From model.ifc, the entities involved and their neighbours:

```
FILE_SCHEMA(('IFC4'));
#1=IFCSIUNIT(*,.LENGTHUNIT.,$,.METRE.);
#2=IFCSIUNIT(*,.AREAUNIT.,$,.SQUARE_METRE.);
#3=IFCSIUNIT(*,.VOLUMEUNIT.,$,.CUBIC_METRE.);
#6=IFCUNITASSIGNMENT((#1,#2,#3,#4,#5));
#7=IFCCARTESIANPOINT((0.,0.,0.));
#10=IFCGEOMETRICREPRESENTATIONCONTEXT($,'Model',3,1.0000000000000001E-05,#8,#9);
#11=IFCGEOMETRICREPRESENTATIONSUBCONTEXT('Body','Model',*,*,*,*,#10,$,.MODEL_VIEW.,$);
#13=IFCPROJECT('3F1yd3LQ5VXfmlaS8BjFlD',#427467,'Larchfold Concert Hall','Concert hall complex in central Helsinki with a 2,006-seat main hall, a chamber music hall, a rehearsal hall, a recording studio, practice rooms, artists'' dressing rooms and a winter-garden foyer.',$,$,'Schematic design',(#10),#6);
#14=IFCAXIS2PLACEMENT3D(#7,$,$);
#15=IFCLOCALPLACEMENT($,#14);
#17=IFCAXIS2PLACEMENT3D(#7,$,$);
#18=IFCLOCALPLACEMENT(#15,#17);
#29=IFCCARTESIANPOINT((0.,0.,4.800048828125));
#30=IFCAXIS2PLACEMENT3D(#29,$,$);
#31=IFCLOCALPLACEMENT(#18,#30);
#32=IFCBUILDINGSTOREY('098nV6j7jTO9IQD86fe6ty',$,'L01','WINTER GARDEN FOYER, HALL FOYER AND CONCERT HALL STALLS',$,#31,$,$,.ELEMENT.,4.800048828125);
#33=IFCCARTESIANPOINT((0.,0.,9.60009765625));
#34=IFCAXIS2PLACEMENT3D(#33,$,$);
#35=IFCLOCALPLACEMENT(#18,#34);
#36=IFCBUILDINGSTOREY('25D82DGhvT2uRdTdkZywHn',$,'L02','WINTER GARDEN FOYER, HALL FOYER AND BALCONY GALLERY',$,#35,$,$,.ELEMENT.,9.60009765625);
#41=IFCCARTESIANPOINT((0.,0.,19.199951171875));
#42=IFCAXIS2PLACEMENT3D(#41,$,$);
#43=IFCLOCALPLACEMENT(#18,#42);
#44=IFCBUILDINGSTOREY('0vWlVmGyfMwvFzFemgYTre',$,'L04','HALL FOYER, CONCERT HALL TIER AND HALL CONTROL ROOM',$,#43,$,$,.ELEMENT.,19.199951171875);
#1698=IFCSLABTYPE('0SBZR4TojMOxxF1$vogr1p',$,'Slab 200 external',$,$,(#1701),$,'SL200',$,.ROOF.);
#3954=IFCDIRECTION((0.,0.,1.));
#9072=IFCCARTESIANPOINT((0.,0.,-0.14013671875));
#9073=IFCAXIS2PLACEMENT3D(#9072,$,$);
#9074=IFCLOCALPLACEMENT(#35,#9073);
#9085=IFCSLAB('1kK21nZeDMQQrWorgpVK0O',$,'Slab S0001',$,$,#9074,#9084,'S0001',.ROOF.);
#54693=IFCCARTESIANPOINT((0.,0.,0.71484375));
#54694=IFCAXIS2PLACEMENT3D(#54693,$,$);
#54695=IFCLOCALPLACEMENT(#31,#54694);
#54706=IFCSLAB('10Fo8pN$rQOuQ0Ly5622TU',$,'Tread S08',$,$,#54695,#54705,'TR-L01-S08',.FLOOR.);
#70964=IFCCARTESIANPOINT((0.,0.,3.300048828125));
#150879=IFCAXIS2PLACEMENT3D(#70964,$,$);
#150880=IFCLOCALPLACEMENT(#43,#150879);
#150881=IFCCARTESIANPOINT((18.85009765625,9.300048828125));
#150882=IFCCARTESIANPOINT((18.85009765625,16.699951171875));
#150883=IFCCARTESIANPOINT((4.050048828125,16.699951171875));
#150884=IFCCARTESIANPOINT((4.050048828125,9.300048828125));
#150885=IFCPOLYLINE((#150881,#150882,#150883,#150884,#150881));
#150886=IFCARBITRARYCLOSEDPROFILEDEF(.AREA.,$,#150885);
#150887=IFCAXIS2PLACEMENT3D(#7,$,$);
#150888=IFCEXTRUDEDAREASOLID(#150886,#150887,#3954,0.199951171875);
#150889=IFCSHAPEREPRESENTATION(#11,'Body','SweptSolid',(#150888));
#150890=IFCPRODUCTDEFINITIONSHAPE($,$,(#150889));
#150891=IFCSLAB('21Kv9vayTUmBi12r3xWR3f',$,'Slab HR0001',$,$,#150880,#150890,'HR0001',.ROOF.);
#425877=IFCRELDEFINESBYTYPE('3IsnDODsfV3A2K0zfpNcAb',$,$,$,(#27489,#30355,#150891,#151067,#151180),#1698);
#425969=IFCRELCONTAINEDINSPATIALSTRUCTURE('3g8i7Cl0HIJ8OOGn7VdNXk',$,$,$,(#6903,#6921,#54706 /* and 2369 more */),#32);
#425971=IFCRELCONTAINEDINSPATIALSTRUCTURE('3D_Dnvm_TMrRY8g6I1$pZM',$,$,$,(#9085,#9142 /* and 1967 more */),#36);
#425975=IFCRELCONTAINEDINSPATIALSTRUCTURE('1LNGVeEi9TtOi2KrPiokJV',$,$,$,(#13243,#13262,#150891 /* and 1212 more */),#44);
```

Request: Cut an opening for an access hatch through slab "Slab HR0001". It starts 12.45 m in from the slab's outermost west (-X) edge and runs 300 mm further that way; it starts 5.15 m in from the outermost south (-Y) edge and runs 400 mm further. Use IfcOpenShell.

```python
import numpy as np
import ifcopenshell
import ifcopenshell.api.feature
import ifcopenshell.api.geometry
import ifcopenshell.api.root
import ifcopenshell.geom
import ifcopenshell.util.placement
import ifcopenshell.util.representation
import ifcopenshell.util.shape
import ifcopenshell.util.unit

model = ifcopenshell.open("model.ifc")
unit_scale = ifcopenshell.util.unit.calculate_unit_scale(model)
settings = ifcopenshell.geom.settings()


def volume(element):
    """Net volume in cubic metres, openings subtracted."""
    shape = ifcopenshell.geom.create_shape(settings, element)
    return ifcopenshell.util.shape.get_volume(shape.geometry)


slab = model.by_guid("21Kv9vayTUmBi12r3xWR3f")
before = volume(slab)

# Extent in the slab's own axes, in metres. The edges named are its -X and -Y sides.
slab_shape = ifcopenshell.geom.create_shape(settings, slab)
vertices = ifcopenshell.util.shape.get_vertices(slab_shape.geometry)
x_min, y_min, bottom = vertices.min(axis=0)
top = vertices[:, 2].max()

opening = ifcopenshell.api.root.create_entity(model, ifc_class="IfcOpeningElement", name="Access hatch opening", predefined_type="OPENING")
context = ifcopenshell.util.representation.get_context(model, "Model", "Body", "MODEL_VIEW")
width, depth = 0.3, 0.4
outline = [(0.0, 0.0), (width, 0.0), (width, depth), (0.0, depth), (0.0, 0.0)]
# Overshoot both faces by 50 mm so the cut is clean.
shape = ifcopenshell.api.geometry.add_slab_representation(
    model, context=context, depth=top - bottom + 0.1, polyline=outline
)
ifcopenshell.api.geometry.assign_representation(model, product=opening, representation=shape)

matrix = ifcopenshell.util.placement.get_local_placement(slab.ObjectPlacement)
matrix[:, 3] = matrix @ np.append(np.array([x_min + 12.45, y_min + 5.15, bottom - 0.05]) / unit_scale, 1.0)
ifcopenshell.api.geometry.edit_object_placement(model, product=opening, matrix=matrix, is_si=False)
ifcopenshell.api.feature.add_feature(model, feature=opening, element=slab)

after = volume(slab)

print(f"slab volume {before:.3f} -> {after:.3f} m3")

model.write("model_edited.ifc")
```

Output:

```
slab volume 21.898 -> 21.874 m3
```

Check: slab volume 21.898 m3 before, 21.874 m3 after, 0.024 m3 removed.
